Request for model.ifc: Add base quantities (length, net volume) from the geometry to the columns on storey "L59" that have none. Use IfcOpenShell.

First a look at what the model holds.

```python
import ifcopenshell
import ifcopenshell.util.element
import ifcopenshell.util.unit

model = ifcopenshell.open("model.ifc")
print(model.schema)
for unit_type in ("LENGTHUNIT", "AREAUNIT", "VOLUMEUNIT"):
    print(unit_type, ifcopenshell.util.unit.calculate_unit_scale(model, unit_type))
storey = next(s for s in model.by_type("IfcBuildingStorey") if s.Name == "L59")
columns = [e for e in ifcopenshell.util.element.get_decomposition(storey) if e.is_a("IfcColumn")]
for e in sorted(columns, key=lambda e: e.id()):
    print(e.id(), e.is_a(), e.Name, list(ifcopenshell.util.element.get_psets(e, qtos_only=True)), sep=" | ")
```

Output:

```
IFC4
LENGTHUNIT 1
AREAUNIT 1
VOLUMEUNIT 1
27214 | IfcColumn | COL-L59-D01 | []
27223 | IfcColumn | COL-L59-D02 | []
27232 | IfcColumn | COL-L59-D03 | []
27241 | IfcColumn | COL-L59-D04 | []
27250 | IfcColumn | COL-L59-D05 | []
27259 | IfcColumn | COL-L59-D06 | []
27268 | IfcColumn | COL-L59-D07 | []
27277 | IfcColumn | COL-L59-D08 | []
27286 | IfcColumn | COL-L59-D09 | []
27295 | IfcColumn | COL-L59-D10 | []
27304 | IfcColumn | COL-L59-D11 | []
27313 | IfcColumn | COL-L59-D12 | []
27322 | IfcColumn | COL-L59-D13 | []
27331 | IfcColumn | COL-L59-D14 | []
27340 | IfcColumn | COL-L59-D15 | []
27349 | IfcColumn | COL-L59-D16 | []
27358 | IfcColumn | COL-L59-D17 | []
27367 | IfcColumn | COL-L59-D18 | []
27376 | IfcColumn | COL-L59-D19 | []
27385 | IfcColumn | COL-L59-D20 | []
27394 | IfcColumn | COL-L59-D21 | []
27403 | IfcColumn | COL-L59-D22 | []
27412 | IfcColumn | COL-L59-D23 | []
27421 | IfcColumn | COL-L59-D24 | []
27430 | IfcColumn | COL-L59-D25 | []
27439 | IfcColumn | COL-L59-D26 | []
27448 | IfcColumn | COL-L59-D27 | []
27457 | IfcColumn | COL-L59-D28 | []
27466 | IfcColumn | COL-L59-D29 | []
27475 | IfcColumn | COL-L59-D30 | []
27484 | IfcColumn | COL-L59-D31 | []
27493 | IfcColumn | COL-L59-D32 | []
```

```python
import ifcopenshell
import ifcopenshell.api.pset
import ifcopenshell.geom
import ifcopenshell.util.element
import ifcopenshell.util.shape
import ifcopenshell.util.unit

model = ifcopenshell.open("model.ifc")
unit_scale = ifcopenshell.util.unit.calculate_unit_scale(model)
volume_scale = ifcopenshell.util.unit.calculate_unit_scale(model, "VOLUMEUNIT")
settings = ifcopenshell.geom.settings()

storey = next(s for s in model.by_type("IfcBuildingStorey") if s.Name == "L59")
columns = [e for e in ifcopenshell.util.element.get_decomposition(storey) if e.is_a("IfcColumn")]

for e in sorted(columns, key=lambda e: e.id()):
    if ifcopenshell.util.element.get_psets(e, qtos_only=True, should_inherit=False):
        continue
    # Geometry comes back in metres, in the element's own axes.
    shape = ifcopenshell.geom.create_shape(settings, e)
    values = {
        "Length": ifcopenshell.util.shape.get_z(shape.geometry) / unit_scale,
        "NetVolume": ifcopenshell.util.shape.get_volume(shape.geometry) / volume_scale,
    }
    qto = ifcopenshell.api.pset.add_qto(model, product=e, name="Qto_ColumnBaseQuantities")
    ifcopenshell.api.pset.edit_qto(model, qto=qto, properties=values)
    print(e.id(), {k: round(v, 3) for k, v in values.items()})

model.write("model_updated.ifc")
```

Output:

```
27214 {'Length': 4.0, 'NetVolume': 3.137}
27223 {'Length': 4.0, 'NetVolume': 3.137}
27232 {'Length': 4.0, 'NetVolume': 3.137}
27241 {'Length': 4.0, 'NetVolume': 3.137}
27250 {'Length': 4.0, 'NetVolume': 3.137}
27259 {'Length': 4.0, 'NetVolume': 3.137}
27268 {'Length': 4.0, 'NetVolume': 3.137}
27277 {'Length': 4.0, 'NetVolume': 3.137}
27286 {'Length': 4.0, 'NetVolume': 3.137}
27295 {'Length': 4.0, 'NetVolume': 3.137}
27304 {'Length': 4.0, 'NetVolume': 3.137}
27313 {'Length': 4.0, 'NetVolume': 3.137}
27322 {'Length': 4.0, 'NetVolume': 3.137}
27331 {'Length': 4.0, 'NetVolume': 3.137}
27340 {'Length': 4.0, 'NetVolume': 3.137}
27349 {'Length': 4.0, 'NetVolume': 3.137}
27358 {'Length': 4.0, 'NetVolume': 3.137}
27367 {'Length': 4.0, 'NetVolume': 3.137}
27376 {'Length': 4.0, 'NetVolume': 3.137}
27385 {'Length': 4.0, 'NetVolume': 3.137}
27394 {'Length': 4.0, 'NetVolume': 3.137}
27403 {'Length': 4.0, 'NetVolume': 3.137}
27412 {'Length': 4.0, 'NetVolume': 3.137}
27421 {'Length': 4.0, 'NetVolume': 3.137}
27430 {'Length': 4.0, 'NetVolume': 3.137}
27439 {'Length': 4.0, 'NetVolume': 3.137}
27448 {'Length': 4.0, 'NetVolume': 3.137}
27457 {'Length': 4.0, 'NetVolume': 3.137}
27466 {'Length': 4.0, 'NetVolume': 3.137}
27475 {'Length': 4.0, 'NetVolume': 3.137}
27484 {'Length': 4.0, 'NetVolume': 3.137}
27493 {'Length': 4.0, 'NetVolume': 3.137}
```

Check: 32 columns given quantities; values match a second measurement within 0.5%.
